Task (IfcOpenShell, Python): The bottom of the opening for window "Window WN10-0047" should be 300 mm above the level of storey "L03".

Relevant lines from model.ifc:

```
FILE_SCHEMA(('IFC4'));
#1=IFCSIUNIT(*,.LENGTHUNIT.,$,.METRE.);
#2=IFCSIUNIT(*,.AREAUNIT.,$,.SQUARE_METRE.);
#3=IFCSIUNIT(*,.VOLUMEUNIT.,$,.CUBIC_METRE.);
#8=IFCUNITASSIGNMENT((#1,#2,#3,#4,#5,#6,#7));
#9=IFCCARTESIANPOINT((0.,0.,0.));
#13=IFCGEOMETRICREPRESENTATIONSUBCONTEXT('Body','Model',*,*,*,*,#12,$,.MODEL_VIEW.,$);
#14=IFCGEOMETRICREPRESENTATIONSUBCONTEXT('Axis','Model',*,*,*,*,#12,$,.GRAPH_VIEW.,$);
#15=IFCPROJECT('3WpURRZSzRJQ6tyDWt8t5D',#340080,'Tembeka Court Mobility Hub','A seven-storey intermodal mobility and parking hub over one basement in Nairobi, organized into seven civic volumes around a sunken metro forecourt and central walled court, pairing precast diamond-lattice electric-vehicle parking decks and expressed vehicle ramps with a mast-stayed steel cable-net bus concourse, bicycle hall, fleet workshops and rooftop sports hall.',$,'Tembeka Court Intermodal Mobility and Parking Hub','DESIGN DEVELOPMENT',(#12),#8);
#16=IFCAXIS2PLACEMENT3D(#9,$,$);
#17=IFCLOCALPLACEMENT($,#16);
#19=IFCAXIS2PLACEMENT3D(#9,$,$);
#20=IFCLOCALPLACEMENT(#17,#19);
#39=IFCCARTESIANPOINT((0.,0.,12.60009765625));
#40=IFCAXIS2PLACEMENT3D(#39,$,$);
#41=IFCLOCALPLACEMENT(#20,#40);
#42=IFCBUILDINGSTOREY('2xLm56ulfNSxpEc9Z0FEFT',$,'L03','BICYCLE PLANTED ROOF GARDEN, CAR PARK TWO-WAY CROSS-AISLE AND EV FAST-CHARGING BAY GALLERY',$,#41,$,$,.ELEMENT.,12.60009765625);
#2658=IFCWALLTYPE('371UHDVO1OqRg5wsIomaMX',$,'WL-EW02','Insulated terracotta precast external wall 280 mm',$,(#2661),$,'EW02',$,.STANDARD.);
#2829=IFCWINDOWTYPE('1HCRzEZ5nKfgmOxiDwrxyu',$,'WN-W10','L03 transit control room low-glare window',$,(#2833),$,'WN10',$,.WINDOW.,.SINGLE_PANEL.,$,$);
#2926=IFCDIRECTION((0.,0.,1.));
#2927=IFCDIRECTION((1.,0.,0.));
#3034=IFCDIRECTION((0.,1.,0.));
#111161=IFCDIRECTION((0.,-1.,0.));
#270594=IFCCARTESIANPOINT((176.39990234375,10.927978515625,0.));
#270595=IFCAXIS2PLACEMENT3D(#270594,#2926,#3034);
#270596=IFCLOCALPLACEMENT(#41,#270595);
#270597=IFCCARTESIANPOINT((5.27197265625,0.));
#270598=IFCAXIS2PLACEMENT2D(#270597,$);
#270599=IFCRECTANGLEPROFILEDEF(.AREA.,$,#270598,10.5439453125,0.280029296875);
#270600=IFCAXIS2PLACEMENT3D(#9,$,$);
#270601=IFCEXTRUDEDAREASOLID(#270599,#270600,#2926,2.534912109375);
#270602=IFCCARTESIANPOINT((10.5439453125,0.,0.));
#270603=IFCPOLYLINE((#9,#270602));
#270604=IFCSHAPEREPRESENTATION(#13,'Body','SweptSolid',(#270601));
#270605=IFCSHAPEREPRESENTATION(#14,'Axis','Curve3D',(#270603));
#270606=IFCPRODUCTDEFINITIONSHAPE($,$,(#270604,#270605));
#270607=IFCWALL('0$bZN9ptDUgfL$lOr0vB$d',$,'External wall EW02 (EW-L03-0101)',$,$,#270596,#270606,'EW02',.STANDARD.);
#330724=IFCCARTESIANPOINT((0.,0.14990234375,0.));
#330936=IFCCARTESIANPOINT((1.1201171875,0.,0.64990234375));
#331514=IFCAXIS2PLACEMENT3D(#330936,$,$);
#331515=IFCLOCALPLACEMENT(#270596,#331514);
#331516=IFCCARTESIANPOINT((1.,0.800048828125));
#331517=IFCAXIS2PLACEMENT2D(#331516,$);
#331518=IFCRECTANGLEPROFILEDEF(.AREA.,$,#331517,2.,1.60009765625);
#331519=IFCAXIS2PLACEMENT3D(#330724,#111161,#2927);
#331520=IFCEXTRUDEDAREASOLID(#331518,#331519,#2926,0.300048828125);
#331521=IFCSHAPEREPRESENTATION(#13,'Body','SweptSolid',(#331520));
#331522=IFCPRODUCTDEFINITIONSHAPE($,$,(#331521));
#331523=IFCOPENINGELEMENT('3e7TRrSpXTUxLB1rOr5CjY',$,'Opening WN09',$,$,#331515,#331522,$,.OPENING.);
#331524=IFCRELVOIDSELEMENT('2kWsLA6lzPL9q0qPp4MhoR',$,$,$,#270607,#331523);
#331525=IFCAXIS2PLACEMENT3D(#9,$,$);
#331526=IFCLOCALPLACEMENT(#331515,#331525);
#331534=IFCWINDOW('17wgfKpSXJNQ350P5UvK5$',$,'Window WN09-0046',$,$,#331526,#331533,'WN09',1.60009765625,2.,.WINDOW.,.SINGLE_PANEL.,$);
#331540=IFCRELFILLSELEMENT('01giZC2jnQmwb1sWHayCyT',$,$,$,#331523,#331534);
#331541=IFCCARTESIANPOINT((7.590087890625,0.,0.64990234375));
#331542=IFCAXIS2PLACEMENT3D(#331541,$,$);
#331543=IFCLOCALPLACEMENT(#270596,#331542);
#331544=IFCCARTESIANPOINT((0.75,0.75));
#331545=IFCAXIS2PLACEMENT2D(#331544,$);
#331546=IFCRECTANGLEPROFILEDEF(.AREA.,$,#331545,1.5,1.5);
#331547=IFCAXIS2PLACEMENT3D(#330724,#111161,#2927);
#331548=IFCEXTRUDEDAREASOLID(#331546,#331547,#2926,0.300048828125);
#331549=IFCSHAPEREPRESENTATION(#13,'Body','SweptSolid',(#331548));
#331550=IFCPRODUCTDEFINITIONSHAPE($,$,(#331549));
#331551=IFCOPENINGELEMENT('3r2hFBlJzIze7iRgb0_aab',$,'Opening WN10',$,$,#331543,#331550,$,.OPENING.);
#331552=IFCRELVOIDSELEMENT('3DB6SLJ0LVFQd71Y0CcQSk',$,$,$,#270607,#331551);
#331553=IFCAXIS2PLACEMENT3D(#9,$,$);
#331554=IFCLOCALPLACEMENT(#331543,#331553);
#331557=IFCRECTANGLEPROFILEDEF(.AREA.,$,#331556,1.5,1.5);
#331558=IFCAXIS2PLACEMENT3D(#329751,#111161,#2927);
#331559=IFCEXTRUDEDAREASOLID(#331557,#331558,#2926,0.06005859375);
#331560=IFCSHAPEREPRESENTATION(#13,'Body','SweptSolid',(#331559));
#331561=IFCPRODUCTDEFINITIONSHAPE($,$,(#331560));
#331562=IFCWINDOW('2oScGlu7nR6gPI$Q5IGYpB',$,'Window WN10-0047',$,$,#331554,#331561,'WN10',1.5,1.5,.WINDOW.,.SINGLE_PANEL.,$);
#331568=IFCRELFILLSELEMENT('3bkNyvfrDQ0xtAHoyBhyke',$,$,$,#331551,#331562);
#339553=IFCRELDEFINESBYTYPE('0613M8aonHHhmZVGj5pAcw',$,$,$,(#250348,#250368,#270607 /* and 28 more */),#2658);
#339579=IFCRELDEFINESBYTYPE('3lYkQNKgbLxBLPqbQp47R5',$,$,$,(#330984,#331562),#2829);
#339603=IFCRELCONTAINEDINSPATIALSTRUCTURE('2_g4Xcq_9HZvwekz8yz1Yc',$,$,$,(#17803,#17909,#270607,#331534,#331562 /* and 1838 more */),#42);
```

```python
import numpy as np
import ifcopenshell
import ifcopenshell.api.geometry
import ifcopenshell.geom
import ifcopenshell.util.element
import ifcopenshell.util.placement
import ifcopenshell.util.shape
import ifcopenshell.util.unit

model = ifcopenshell.open("model.ifc")
unit_scale = ifcopenshell.util.unit.calculate_unit_scale(model)

window = model.by_guid("2oScGlu7nR6gPI$Q5IGYpB")
opening = window.FillsVoids[0].RelatingOpeningElement
storey = ifcopenshell.util.element.get_container(window, ifc_class="IfcBuildingStorey")
level = ifcopenshell.util.placement.get_local_placement(storey.ObjectPlacement)[2, 3]

# The opening's origin need not be at the sill, so measure its lowest point.
shape = ifcopenshell.geom.create_shape(ifcopenshell.geom.settings(), opening)
bottom = ifcopenshell.util.shape.get_shape_bottom_elevation(shape, shape.geometry) / unit_scale
dz = level + 0.3 - bottom

shift = np.array([0.0, 0.0, dz])
# The window is placed relative to its opening, so it follows when the opening moves.
matrix = ifcopenshell.util.placement.get_local_placement(opening.ObjectPlacement)
matrix[:3, 3] += shift
ifcopenshell.api.geometry.edit_object_placement(
    model, product=opening, matrix=matrix, is_si=False, should_transform_children=True
)

print(f"moved by {dz * unit_scale:+.3f} m")

model.write("model-out.ifc")
```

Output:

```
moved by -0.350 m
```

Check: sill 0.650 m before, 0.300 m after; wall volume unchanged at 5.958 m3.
